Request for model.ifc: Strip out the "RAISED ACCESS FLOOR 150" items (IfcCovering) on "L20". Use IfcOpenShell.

First a look at what the model holds.

```python
import ifcopenshell
import ifcopenshell.util.element

model = ifcopenshell.open("model.ifc")
print(model.schema)
storey = next(s for s in model.by_type("IfcBuildingStorey") if s.Name == "L20")
coverings = [e for e in ifcopenshell.util.element.get_decomposition(storey) if e.is_a("IfcCovering")]
seen = {}
for e in coverings:
    element_type = ifcopenshell.util.element.get_type(e)
    name = element_type.Name if element_type not in (None, e) else None
    seen[name] = seen.get(name, 0) + 1
for name, count in sorted(seen.items(), key=str):
    print(count, "x", name)
```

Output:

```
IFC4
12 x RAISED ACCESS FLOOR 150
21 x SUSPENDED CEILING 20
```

```python
import ifcopenshell
import ifcopenshell.api.root
import ifcopenshell.util.element

model = ifcopenshell.open("model.ifc")

storey = next(s for s in model.by_type("IfcBuildingStorey") if s.Name == "L20")
coverings = [e for e in ifcopenshell.util.element.get_decomposition(storey) if e.is_a("IfcCovering")]
targets = [e for e in coverings if (t := ifcopenshell.util.element.get_type(e)) not in (None, e) and t.Name == "RAISED ACCESS FLOOR 150"]

for e in targets:
    ifcopenshell.api.root.remove_product(model, product=e)
print(len(targets), "removed")

model.write("model_edited.ifc")
```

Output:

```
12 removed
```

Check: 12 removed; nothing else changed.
